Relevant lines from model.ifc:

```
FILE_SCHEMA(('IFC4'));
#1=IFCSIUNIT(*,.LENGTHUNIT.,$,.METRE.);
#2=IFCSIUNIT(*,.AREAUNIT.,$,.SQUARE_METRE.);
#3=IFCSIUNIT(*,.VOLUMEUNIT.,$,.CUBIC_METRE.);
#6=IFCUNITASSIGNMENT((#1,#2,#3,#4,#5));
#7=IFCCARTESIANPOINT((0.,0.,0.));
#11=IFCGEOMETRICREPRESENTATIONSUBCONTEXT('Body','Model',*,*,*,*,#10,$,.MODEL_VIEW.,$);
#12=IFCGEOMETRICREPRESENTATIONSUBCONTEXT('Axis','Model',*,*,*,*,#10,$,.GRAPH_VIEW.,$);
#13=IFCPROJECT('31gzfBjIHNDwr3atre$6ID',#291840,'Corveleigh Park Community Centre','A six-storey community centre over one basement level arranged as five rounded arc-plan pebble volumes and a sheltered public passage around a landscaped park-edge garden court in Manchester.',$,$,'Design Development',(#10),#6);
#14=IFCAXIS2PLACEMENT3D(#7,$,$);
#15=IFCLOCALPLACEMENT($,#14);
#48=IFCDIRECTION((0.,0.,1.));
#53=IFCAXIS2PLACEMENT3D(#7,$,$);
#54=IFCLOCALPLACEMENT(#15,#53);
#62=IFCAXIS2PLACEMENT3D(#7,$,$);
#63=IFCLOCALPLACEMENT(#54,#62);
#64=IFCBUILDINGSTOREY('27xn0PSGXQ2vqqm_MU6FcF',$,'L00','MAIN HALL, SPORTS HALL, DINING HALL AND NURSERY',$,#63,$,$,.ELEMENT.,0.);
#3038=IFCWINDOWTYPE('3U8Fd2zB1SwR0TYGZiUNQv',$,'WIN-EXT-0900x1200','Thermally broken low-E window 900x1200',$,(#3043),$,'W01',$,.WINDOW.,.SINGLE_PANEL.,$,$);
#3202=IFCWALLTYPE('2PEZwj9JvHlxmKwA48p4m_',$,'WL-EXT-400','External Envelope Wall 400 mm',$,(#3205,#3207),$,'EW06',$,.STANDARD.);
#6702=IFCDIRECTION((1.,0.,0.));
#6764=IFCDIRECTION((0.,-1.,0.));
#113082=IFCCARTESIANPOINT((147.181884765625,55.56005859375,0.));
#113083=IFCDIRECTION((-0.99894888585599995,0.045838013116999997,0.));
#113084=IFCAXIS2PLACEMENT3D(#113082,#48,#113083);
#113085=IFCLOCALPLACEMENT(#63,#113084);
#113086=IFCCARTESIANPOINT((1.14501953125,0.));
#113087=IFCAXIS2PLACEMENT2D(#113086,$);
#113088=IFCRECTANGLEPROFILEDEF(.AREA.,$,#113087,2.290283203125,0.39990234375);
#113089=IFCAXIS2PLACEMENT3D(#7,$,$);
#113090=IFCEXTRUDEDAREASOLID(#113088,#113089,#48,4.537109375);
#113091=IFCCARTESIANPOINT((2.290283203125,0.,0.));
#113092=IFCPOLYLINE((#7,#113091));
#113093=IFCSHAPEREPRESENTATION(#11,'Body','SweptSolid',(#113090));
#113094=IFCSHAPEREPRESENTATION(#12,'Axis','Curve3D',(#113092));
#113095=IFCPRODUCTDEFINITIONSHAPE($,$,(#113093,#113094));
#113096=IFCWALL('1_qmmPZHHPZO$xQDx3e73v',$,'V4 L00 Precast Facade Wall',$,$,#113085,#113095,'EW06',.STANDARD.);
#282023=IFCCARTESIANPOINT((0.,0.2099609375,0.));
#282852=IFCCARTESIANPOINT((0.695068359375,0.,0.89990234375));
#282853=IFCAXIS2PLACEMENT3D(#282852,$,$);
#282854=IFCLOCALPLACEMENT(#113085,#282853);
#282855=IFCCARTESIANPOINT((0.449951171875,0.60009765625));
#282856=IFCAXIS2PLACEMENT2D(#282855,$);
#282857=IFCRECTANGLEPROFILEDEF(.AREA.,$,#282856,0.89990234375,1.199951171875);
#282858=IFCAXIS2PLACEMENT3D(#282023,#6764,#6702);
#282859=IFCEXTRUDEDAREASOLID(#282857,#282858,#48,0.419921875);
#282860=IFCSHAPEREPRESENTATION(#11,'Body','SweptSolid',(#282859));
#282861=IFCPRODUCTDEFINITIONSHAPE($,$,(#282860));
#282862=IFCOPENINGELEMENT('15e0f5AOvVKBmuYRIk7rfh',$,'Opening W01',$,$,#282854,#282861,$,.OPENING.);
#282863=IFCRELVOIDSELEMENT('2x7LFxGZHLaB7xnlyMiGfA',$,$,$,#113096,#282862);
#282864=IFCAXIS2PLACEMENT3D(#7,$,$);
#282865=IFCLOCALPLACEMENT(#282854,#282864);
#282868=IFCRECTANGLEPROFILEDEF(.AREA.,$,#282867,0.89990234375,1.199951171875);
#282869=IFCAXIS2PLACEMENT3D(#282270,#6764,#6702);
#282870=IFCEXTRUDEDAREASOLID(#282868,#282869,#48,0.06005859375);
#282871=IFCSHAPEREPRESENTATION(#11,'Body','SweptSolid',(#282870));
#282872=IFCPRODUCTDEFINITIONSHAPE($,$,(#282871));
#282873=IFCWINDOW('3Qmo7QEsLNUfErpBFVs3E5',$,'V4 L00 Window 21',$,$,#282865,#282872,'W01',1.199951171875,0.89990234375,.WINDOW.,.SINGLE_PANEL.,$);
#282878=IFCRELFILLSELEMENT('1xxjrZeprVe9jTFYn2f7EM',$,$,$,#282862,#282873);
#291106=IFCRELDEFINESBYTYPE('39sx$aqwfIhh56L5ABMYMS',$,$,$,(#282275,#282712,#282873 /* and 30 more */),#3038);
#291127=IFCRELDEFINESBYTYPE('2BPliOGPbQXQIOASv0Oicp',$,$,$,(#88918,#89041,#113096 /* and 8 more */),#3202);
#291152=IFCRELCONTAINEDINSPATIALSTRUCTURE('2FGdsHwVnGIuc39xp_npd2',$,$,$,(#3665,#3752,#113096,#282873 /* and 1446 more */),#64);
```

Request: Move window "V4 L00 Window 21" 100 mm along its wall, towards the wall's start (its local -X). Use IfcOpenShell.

```python
import ifcopenshell
import ifcopenshell.api.geometry
import ifcopenshell.util.placement
import ifcopenshell.util.unit

model = ifcopenshell.open("model.ifc")
unit_scale = ifcopenshell.util.unit.calculate_unit_scale(model)

window = model.by_id(282873)
opening = window.FillsVoids[0].RelatingOpeningElement
wall = opening.VoidsElements[0].RelatingBuildingElement

wall_matrix = ifcopenshell.util.placement.get_local_placement(wall.ObjectPlacement)
shift = wall_matrix[:3, 0] * -0.1 / unit_scale
before = ifcopenshell.util.placement.get_local_placement(window.ObjectPlacement)[:3, 3].copy()

# The window is placed relative to its opening, so it follows when the opening moves.
matrix = ifcopenshell.util.placement.get_local_placement(opening.ObjectPlacement)
matrix[:3, 3] += shift
ifcopenshell.api.geometry.edit_object_placement(
    model, product=opening, matrix=matrix, is_si=False, should_transform_children=True
)

after = ifcopenshell.util.placement.get_local_placement(window.ObjectPlacement)[:3, 3]
print("window moved by", (after - before).round(3) + 0.0)

model.write("model-out.ifc")
```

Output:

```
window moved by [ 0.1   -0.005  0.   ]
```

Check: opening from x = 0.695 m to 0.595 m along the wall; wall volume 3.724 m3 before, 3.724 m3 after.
